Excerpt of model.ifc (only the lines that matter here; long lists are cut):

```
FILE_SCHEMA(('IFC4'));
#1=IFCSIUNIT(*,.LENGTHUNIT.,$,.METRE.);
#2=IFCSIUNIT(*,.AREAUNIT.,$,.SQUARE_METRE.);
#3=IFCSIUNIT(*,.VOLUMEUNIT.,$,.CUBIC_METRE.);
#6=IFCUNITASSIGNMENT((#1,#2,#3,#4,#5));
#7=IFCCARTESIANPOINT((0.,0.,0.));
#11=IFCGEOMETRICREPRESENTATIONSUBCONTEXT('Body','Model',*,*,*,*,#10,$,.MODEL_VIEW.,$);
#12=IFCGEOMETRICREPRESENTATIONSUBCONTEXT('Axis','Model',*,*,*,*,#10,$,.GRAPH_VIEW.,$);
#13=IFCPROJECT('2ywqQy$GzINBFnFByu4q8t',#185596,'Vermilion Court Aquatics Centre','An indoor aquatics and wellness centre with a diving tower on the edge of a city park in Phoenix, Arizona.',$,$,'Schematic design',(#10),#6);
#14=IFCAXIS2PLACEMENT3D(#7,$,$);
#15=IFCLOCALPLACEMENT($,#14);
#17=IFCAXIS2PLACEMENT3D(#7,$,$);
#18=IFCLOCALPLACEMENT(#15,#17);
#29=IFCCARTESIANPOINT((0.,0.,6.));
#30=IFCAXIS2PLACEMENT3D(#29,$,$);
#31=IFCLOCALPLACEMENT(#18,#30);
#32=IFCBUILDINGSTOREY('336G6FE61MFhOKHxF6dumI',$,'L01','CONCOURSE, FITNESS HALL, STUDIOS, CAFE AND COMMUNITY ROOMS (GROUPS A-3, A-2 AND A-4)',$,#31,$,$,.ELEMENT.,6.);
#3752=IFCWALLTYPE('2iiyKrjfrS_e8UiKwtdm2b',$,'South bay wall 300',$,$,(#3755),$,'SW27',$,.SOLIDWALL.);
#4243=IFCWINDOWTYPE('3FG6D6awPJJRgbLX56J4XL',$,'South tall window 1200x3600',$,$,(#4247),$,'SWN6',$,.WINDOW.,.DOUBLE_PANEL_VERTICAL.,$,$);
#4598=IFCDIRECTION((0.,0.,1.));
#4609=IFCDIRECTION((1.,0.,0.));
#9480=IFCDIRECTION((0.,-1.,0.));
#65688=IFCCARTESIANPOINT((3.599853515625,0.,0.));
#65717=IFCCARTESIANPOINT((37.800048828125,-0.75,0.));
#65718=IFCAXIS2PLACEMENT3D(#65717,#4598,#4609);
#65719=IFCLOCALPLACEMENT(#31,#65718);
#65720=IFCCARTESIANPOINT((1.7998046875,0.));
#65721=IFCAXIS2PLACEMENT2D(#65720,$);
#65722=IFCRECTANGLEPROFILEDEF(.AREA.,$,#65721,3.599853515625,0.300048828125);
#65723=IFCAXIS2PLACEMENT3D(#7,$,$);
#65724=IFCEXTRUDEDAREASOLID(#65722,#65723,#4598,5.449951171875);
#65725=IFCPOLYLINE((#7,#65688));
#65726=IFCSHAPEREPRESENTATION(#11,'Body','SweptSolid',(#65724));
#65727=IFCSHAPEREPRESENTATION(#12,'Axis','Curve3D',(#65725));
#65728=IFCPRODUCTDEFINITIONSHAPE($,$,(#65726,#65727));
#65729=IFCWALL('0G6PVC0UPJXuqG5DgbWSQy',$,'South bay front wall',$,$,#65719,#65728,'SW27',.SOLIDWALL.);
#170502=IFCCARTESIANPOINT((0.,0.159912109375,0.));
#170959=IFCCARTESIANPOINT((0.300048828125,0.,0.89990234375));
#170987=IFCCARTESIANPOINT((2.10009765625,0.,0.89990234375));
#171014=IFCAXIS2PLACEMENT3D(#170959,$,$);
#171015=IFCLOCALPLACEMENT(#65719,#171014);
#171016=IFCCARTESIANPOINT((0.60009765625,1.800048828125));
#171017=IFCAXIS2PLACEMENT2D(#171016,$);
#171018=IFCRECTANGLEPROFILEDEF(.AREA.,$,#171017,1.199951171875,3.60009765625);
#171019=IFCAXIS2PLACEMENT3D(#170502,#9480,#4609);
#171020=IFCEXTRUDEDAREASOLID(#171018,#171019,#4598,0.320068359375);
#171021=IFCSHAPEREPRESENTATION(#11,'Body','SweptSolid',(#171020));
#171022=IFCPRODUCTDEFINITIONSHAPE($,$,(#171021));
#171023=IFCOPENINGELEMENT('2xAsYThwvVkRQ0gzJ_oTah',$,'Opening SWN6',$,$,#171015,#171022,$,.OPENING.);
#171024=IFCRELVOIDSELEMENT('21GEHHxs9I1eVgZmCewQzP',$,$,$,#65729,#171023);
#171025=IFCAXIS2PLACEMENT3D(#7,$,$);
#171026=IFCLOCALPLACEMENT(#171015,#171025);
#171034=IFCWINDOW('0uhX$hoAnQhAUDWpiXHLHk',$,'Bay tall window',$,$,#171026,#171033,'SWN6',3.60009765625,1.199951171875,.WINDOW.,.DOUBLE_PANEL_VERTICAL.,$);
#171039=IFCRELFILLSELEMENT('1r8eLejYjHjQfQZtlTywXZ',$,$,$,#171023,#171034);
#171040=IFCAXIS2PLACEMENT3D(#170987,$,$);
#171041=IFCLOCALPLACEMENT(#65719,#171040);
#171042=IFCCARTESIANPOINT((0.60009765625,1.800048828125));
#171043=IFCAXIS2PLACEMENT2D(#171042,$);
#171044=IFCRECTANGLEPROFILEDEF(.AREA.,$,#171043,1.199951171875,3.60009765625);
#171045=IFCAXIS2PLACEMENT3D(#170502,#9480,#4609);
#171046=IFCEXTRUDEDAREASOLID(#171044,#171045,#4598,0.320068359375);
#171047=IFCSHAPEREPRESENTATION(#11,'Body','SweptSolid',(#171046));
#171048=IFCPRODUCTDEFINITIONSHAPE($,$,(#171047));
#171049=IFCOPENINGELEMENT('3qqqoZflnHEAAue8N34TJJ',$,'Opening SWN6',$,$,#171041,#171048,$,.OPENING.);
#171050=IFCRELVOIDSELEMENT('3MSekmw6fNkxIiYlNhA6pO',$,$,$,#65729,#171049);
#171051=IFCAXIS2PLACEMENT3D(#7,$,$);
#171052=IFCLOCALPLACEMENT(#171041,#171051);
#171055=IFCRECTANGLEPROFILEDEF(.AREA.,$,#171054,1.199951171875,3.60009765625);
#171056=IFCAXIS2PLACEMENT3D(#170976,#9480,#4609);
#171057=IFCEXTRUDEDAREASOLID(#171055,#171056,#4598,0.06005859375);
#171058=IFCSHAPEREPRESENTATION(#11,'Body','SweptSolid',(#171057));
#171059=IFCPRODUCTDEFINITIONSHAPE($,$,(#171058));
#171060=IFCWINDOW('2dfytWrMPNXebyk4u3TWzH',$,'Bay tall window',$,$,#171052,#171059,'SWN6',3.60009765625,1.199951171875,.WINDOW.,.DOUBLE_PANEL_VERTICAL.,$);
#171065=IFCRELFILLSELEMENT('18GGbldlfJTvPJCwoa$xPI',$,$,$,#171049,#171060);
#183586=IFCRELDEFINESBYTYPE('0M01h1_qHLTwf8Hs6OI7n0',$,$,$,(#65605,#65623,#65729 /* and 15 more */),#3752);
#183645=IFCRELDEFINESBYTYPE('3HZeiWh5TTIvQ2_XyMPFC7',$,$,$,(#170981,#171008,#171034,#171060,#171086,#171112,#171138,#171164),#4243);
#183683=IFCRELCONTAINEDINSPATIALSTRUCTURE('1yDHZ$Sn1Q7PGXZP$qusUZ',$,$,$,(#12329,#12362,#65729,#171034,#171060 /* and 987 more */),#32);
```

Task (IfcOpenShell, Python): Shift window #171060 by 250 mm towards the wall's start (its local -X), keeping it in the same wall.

```python
import ifcopenshell
import ifcopenshell.api.geometry
import ifcopenshell.util.placement
import ifcopenshell.util.unit

model = ifcopenshell.open("model.ifc")
unit_scale = ifcopenshell.util.unit.calculate_unit_scale(model)

window = model.by_id(171060)
opening = window.FillsVoids[0].RelatingOpeningElement
wall = opening.VoidsElements[0].RelatingBuildingElement

wall_matrix = ifcopenshell.util.placement.get_local_placement(wall.ObjectPlacement)
shift = wall_matrix[:3, 0] * -0.25 / unit_scale
before = ifcopenshell.util.placement.get_local_placement(window.ObjectPlacement)[:3, 3].copy()

# The window is placed relative to its opening, so it follows when the opening moves.
matrix = ifcopenshell.util.placement.get_local_placement(opening.ObjectPlacement)
matrix[:3, 3] += shift
ifcopenshell.api.geometry.edit_object_placement(
    model, product=opening, matrix=matrix, is_si=False, should_transform_children=True
)

after = ifcopenshell.util.placement.get_local_placement(window.ObjectPlacement)[:3, 3]
print("window moved by", (after - before).round(3) + 0.0)

model.write("model_edited.ifc")
```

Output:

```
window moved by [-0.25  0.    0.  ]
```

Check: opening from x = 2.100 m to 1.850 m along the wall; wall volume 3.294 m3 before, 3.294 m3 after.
